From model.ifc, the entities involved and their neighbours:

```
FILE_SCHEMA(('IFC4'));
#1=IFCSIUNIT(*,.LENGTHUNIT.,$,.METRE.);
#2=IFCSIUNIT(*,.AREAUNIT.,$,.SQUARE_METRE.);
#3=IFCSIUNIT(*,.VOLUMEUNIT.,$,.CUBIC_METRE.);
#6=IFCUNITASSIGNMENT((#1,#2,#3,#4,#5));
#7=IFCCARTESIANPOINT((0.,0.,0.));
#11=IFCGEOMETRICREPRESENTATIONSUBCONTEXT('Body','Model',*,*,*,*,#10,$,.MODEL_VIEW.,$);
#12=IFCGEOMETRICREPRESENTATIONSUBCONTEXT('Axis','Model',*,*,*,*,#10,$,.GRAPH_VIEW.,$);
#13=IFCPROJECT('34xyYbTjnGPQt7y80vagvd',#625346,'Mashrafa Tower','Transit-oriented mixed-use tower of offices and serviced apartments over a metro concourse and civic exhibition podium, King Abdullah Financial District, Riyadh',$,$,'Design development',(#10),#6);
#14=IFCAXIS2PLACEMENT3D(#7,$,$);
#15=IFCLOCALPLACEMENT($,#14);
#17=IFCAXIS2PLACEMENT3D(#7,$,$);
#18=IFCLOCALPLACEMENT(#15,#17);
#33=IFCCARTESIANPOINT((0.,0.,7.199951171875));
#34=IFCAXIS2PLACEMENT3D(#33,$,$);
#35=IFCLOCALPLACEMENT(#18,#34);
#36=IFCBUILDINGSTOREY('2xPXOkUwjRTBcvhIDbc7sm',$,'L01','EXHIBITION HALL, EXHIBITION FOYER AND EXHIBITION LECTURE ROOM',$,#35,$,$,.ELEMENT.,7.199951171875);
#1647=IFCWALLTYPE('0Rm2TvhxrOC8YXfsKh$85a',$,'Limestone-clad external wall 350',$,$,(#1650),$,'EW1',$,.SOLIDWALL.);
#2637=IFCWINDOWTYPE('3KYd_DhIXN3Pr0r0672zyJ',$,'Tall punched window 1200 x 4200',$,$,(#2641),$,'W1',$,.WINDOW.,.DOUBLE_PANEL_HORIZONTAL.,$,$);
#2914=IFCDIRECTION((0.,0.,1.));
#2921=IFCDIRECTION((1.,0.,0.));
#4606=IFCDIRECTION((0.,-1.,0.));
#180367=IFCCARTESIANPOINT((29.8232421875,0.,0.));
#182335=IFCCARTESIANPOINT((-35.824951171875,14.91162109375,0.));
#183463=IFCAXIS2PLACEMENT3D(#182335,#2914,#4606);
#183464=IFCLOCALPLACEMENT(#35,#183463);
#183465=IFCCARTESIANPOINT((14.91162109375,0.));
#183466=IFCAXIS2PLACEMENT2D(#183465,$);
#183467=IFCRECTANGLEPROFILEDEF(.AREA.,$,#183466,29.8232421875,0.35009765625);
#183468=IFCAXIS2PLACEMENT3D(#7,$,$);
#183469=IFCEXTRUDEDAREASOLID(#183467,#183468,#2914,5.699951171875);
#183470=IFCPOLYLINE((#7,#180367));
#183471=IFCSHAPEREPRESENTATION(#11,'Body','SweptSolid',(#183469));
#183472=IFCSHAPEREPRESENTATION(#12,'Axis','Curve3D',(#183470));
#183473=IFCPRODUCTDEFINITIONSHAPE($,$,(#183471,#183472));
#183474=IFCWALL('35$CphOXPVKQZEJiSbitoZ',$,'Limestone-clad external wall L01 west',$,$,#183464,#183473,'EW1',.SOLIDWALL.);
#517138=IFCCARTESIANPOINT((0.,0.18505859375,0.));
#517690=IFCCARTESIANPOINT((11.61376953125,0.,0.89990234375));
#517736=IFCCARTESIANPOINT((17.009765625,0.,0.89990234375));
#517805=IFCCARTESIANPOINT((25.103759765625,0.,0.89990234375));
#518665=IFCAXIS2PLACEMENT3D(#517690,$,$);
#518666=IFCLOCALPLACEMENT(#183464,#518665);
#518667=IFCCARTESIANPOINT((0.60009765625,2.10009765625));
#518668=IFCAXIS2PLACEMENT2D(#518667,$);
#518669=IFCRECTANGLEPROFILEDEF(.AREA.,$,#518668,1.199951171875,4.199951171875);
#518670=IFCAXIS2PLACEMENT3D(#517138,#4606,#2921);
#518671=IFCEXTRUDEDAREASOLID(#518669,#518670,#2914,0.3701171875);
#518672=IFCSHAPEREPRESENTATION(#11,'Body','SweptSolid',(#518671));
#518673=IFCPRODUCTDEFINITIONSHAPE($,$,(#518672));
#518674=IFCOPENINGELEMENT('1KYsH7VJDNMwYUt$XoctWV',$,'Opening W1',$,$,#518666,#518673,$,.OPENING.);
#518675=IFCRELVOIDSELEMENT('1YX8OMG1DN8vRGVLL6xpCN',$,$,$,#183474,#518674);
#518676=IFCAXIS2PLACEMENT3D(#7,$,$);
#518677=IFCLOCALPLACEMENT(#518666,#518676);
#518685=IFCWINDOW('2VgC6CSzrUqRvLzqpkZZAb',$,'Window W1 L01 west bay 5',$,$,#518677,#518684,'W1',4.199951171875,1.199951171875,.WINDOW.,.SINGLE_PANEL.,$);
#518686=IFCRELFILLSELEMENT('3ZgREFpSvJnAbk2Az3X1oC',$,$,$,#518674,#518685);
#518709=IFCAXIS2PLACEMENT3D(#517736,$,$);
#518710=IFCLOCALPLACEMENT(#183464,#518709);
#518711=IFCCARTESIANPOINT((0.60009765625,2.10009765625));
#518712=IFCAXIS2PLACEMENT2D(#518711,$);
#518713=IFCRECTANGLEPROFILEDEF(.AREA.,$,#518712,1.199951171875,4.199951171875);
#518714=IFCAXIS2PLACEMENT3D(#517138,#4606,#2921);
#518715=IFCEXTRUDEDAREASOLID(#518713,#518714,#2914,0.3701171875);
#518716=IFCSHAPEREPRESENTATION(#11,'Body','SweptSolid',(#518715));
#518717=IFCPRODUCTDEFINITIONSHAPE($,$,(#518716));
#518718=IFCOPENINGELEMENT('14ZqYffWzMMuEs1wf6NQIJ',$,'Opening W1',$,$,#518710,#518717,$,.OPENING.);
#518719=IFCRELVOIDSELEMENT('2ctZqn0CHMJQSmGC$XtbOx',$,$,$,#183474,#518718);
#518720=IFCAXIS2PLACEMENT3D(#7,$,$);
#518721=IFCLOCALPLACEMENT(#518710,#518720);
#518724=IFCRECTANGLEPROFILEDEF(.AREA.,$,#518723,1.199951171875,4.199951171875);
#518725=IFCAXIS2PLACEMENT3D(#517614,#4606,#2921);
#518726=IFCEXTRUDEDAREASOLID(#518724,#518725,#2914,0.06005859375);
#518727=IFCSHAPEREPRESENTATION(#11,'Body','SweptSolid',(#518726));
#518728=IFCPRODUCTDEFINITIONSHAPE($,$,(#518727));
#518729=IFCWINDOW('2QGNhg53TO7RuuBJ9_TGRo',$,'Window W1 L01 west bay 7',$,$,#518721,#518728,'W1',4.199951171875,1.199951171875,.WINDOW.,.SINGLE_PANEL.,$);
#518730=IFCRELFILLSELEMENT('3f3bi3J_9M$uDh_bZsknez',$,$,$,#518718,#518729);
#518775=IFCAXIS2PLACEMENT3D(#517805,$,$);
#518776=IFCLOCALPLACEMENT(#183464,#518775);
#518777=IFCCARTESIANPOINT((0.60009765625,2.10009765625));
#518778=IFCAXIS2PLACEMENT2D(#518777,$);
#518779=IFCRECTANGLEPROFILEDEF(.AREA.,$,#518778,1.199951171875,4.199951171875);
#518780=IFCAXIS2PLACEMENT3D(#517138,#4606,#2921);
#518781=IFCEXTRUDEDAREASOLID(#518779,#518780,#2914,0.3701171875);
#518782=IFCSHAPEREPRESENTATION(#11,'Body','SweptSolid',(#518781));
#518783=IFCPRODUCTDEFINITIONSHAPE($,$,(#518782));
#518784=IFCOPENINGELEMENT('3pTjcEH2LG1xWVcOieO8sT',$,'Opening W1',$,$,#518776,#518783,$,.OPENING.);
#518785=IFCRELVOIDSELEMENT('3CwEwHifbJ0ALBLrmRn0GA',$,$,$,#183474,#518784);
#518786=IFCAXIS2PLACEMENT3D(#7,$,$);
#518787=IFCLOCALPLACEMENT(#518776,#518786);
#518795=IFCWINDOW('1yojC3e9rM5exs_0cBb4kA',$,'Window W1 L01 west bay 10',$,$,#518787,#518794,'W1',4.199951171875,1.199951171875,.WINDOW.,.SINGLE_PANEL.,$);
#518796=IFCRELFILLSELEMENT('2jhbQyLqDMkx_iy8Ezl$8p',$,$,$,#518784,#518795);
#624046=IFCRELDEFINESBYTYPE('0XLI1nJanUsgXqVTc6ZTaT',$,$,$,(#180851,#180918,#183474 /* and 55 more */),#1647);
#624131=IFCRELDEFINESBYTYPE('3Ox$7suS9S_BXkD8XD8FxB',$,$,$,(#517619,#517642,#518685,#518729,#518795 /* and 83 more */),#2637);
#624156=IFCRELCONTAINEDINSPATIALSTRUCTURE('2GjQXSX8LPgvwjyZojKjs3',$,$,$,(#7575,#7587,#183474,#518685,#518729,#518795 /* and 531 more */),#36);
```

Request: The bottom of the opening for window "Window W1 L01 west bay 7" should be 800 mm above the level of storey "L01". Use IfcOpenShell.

```python
import numpy as np
import ifcopenshell
import ifcopenshell.api.geometry
import ifcopenshell.geom
import ifcopenshell.util.element
import ifcopenshell.util.placement
import ifcopenshell.util.shape
import ifcopenshell.util.unit

model = ifcopenshell.open("model.ifc")
unit_scale = ifcopenshell.util.unit.calculate_unit_scale(model)

window = model.by_guid("2QGNhg53TO7RuuBJ9_TGRo")
opening = window.FillsVoids[0].RelatingOpeningElement
storey = ifcopenshell.util.element.get_container(window, ifc_class="IfcBuildingStorey")
level = ifcopenshell.util.placement.get_local_placement(storey.ObjectPlacement)[2, 3]

# The opening's origin need not be at the sill, so measure its lowest point.
shape = ifcopenshell.geom.create_shape(ifcopenshell.geom.settings(), opening)
bottom = ifcopenshell.util.shape.get_shape_bottom_elevation(shape, shape.geometry) / unit_scale
dz = level + 0.8 / unit_scale - bottom

shift = np.array([0.0, 0.0, dz])
# The window is placed relative to its opening, so it follows when the opening moves.
matrix = ifcopenshell.util.placement.get_local_placement(opening.ObjectPlacement)
matrix[:3, 3] += shift
ifcopenshell.api.geometry.edit_object_placement(
    model, product=opening, matrix=matrix, is_si=False, should_transform_children=True
)

print(f"moved by {dz * unit_scale:+.3f} m")

model.write("model_edited.ifc")
```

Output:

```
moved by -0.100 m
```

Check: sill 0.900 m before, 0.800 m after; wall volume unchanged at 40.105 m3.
